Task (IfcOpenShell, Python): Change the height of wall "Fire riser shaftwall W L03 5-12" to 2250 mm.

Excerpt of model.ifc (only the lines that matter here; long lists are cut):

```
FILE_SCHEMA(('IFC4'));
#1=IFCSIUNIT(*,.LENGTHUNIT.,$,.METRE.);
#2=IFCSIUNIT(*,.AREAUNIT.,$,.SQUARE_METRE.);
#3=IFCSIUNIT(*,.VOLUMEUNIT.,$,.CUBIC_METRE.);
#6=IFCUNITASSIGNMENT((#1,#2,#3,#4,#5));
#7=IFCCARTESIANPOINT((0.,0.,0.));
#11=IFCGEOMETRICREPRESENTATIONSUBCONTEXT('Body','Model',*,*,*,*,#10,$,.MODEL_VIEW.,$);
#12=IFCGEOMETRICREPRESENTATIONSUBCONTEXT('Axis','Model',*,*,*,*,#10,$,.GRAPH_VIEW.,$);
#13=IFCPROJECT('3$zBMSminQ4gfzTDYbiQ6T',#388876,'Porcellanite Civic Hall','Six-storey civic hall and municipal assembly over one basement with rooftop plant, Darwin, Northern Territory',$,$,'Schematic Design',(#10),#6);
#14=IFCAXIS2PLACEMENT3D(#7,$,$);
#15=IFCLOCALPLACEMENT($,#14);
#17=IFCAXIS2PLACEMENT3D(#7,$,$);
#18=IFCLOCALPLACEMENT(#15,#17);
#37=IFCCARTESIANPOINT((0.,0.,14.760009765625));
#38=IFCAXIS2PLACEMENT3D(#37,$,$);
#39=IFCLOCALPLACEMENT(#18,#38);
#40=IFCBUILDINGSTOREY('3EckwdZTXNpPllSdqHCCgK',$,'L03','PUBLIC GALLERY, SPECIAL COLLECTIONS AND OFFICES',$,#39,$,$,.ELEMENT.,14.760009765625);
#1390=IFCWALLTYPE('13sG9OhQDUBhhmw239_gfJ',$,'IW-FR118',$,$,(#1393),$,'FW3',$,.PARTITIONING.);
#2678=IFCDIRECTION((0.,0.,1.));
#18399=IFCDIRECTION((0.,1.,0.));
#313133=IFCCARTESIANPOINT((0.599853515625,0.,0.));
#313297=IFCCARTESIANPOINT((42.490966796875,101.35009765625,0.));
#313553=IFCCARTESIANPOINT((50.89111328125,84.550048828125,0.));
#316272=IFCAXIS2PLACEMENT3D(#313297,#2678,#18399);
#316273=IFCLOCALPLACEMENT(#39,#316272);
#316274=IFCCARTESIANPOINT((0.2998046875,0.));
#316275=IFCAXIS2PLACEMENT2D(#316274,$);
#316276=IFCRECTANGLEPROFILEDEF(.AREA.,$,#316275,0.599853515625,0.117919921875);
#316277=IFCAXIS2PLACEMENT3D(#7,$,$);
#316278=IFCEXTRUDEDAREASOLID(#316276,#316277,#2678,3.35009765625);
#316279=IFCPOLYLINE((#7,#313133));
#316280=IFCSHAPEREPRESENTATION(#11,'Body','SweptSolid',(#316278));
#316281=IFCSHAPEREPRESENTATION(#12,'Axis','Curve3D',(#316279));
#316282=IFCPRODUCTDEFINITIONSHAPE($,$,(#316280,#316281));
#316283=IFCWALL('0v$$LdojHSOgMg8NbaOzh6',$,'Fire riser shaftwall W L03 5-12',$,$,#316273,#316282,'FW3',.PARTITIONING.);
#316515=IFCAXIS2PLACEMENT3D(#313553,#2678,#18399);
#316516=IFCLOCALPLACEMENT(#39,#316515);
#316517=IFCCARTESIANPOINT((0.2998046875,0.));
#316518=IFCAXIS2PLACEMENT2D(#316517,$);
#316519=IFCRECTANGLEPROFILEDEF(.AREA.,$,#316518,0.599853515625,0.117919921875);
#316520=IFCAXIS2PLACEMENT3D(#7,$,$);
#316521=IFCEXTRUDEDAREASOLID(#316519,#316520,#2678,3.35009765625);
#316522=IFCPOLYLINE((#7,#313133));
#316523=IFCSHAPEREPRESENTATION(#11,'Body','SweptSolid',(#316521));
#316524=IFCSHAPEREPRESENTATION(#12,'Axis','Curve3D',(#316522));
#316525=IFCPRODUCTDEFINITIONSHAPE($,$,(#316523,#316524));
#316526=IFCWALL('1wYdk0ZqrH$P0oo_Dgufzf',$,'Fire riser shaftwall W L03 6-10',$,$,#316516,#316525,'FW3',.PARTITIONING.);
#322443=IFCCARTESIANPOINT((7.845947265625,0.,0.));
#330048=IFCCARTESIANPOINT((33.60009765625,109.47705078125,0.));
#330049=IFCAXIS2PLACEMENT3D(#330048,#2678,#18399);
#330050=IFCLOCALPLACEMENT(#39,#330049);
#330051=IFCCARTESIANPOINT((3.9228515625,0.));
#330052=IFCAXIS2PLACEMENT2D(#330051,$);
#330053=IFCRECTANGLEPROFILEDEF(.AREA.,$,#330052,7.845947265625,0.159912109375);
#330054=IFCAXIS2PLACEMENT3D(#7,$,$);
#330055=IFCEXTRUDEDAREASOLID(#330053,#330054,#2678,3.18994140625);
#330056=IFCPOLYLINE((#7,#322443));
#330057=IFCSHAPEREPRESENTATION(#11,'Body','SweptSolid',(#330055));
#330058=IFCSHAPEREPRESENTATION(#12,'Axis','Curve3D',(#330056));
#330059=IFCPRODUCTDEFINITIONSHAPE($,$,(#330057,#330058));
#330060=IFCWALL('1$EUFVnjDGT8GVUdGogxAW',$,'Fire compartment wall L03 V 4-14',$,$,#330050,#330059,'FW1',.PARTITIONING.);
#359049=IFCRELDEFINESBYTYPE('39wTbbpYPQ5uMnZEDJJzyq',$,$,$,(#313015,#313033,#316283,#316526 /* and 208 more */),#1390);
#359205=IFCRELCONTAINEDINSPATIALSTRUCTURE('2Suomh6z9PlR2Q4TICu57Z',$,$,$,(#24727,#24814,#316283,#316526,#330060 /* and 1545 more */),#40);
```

```python
import ifcopenshell
import ifcopenshell.geom
import ifcopenshell.util.representation
import ifcopenshell.util.shape

model = ifcopenshell.open("model.ifc")
settings = ifcopenshell.geom.settings()


def volume(element):
    """Net volume in cubic metres, openings subtracted."""
    shape = ifcopenshell.geom.create_shape(settings, element)
    return ifcopenshell.util.shape.get_volume(shape.geometry)


wall = model.by_id(316283)
before = volume(wall)

body = ifcopenshell.util.representation.get_representation(wall, "Model", "Body")
solid = body.Items[0]
old_height = solid.Depth
solid.Depth = 2.25
after = volume(wall)

print(f"height {old_height:g} -> {solid.Depth:g}, volume {before:.3f} -> {after:.3f} m3")

model.write("model_v2.ifc")
```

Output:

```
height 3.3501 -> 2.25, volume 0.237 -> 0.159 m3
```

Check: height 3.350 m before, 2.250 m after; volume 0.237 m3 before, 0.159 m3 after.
